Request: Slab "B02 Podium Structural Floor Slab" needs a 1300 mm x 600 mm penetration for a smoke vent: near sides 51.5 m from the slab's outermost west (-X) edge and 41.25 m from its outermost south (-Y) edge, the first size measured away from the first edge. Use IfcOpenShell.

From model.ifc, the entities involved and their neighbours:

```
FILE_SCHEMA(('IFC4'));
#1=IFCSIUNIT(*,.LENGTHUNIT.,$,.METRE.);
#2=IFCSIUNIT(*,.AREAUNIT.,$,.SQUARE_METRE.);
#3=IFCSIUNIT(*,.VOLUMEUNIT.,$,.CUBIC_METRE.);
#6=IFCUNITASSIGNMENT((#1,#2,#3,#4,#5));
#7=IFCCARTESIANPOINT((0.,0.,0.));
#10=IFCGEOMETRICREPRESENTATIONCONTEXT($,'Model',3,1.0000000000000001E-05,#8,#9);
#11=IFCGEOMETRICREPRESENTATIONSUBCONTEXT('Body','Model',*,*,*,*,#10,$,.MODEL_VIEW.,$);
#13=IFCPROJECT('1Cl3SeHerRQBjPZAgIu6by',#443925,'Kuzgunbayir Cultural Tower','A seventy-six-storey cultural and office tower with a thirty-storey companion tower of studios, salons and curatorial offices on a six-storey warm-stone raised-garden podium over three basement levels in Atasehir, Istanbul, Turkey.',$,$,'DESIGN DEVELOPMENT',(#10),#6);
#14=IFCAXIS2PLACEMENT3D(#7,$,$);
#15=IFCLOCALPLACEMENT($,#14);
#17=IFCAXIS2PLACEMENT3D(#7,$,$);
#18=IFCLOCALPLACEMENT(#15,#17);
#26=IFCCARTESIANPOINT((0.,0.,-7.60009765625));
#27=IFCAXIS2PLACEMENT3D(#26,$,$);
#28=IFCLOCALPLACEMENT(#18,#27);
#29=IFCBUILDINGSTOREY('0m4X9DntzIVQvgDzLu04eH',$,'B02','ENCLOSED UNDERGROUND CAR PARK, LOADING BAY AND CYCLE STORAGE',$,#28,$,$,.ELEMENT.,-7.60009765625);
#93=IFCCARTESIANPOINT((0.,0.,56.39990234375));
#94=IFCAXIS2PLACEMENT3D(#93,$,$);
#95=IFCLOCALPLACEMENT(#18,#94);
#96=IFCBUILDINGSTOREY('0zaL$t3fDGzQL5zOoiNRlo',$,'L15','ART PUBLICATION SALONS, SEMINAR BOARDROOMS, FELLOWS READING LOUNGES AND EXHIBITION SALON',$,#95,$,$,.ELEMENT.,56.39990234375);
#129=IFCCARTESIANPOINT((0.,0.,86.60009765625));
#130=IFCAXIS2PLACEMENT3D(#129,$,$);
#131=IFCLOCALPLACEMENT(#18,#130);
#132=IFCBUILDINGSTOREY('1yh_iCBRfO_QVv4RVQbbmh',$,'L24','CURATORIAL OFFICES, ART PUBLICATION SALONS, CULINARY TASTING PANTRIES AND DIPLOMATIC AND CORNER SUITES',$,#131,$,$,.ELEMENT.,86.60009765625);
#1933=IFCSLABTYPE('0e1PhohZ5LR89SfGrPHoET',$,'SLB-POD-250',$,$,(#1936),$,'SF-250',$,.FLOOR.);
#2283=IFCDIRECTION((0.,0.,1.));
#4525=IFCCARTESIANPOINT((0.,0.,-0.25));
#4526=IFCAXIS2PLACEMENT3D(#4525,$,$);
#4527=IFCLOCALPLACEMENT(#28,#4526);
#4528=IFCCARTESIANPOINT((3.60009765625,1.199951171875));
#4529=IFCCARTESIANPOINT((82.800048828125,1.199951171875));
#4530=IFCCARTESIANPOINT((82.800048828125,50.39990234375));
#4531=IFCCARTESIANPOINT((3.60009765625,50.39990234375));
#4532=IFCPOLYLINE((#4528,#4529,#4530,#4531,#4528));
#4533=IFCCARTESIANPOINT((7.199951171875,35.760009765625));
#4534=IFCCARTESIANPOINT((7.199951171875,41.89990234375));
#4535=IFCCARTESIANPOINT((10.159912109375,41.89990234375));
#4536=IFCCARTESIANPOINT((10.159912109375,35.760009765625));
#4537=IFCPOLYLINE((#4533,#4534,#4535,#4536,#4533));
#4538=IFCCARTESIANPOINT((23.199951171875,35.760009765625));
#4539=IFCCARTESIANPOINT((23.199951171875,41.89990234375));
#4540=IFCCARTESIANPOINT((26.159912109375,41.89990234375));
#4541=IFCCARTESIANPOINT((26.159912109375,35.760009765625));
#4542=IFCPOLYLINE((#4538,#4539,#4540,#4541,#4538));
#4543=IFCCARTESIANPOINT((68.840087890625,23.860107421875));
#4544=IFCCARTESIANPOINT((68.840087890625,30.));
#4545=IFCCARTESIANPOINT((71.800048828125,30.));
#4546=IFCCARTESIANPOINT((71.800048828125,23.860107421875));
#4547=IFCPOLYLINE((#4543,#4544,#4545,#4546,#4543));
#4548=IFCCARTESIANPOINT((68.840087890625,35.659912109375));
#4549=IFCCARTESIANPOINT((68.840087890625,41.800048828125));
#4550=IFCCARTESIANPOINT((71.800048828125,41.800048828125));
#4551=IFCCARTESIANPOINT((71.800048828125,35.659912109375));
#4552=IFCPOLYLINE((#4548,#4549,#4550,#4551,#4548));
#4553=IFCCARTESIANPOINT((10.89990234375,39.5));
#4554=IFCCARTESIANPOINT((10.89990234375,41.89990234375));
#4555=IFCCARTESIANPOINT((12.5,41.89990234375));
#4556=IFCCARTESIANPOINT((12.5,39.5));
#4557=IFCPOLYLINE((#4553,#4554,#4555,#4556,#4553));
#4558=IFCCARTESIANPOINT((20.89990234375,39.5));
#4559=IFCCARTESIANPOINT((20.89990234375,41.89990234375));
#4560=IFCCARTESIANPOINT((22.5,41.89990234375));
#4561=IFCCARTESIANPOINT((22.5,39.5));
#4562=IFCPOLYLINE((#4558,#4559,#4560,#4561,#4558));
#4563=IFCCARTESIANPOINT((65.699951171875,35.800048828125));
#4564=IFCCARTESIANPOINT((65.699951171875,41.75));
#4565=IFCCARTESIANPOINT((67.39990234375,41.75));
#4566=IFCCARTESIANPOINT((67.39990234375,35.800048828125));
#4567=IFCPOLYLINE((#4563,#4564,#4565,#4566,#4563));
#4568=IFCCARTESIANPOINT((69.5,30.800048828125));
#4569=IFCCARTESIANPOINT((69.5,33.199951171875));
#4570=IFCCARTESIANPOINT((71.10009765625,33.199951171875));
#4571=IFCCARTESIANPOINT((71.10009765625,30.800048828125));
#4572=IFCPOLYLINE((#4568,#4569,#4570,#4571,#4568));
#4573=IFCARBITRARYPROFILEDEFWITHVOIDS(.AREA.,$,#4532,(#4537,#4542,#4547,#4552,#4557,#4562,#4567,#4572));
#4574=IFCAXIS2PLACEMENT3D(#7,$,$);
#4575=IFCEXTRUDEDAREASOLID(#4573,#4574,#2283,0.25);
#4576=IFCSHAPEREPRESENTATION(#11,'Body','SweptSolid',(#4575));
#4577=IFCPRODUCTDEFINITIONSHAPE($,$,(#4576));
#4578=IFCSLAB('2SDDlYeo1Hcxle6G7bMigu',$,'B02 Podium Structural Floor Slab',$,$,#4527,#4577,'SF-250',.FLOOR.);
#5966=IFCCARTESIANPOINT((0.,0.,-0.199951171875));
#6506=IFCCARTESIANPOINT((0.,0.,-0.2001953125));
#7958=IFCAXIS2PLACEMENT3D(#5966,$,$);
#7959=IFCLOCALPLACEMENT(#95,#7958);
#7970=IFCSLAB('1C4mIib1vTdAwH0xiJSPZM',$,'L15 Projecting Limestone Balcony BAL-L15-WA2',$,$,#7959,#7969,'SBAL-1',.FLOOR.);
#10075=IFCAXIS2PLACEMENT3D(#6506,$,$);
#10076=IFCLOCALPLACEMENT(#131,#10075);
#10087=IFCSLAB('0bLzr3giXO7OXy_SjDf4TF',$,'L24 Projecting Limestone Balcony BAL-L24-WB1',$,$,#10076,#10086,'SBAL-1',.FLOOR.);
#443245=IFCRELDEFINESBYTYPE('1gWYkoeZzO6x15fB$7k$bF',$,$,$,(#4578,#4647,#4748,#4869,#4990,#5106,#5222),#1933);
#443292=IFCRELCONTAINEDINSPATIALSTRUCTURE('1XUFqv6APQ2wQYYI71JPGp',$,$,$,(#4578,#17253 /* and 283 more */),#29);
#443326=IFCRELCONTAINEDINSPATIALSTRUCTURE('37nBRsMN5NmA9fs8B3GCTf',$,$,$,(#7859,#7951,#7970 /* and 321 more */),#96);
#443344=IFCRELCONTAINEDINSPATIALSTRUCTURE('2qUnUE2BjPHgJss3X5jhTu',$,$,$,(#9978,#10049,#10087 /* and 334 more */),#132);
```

```python
import numpy as np
import ifcopenshell
import ifcopenshell.api.feature
import ifcopenshell.api.geometry
import ifcopenshell.api.root
import ifcopenshell.geom
import ifcopenshell.util.placement
import ifcopenshell.util.representation
import ifcopenshell.util.shape
import ifcopenshell.util.unit

model = ifcopenshell.open("model.ifc")
unit_scale = ifcopenshell.util.unit.calculate_unit_scale(model)
settings = ifcopenshell.geom.settings()


def volume(element):
    """Net volume in cubic metres, openings subtracted."""
    shape = ifcopenshell.geom.create_shape(settings, element)
    return ifcopenshell.util.shape.get_volume(shape.geometry)


slab = model.by_guid("2SDDlYeo1Hcxle6G7bMigu")
before = volume(slab)

# Extent in the slab's own axes, in metres. The edges named are its -X and -Y sides.
slab_shape = ifcopenshell.geom.create_shape(settings, slab)
vertices = ifcopenshell.util.shape.get_vertices(slab_shape.geometry)
x_min, y_min, bottom = vertices.min(axis=0)
top = vertices[:, 2].max()

opening = ifcopenshell.api.root.create_entity(model, ifc_class="IfcOpeningElement", name="Smoke vent opening", predefined_type="OPENING")
context = ifcopenshell.util.representation.get_context(model, "Model", "Body", "MODEL_VIEW")
width, depth = 1.3, 0.6
outline = [(0.0, 0.0), (width, 0.0), (width, depth), (0.0, depth), (0.0, 0.0)]
# Overshoot both faces by 50 mm so the cut is clean.
shape = ifcopenshell.api.geometry.add_slab_representation(
    model, context=context, depth=top - bottom + 0.1, polyline=outline
)
ifcopenshell.api.geometry.assign_representation(model, product=opening, representation=shape)

matrix = ifcopenshell.util.placement.get_local_placement(slab.ObjectPlacement)
matrix[:, 3] = matrix @ np.append(np.array([x_min + 51.5, y_min + 41.25, bottom - 0.05]) / unit_scale, 1.0)
ifcopenshell.api.geometry.edit_object_placement(model, product=opening, matrix=matrix, is_si=False)
ifcopenshell.api.feature.add_feature(model, feature=opening, element=slab)

after = volume(slab)

print(f"slab volume {before:.3f} -> {after:.3f} m3")

model.write("model_rev.ifc")
```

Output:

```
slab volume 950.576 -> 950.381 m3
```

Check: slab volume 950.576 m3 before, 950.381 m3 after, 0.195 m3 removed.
